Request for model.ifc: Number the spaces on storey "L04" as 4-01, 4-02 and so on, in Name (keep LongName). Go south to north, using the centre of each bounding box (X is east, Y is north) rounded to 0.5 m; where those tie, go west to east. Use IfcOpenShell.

First a look at what the model holds.

```python
import ifcopenshell
import ifcopenshell.util.element
import ifcopenshell.util.placement

model = ifcopenshell.open("model.ifc")
print(model.schema)
storey = next(s for s in model.by_type("IfcBuildingStorey") if s.Name == "L04")
spaces = [e for e in ifcopenshell.util.element.get_decomposition(storey) if e.is_a("IfcSpace")]
for e in sorted(spaces, key=lambda e: e.id()):
    origin = ifcopenshell.util.placement.get_local_placement(e.ObjectPlacement)[:3, 3]
    print(e.id(), e.Name, e.LongName, origin.round(2) + 0.0, sep=" | ")
```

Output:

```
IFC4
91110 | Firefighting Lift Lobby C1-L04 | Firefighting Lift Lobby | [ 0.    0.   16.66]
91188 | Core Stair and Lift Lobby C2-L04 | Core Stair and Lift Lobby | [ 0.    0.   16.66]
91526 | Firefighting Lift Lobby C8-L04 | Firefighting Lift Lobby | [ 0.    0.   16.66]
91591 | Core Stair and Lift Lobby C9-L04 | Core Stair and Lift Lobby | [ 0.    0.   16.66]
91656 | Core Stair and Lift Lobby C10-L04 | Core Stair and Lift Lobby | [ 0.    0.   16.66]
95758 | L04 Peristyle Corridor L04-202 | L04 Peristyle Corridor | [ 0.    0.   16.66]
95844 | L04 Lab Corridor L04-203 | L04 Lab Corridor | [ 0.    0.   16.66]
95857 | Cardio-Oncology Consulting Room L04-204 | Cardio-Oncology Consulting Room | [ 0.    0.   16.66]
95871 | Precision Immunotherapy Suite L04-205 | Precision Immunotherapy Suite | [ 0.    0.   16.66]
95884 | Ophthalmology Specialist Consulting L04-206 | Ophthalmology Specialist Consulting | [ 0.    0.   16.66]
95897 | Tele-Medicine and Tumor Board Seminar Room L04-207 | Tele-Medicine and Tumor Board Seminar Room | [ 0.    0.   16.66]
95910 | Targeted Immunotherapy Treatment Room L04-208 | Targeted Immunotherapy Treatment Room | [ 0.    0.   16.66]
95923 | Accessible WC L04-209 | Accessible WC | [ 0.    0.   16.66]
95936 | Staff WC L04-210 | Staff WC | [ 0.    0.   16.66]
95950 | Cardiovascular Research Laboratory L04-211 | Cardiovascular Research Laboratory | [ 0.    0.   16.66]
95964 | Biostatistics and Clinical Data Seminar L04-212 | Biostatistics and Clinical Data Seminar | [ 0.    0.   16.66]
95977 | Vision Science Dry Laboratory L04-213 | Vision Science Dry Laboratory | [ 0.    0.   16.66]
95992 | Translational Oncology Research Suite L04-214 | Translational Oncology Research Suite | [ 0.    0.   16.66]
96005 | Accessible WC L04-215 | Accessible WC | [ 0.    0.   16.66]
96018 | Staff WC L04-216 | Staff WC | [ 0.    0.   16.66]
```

```python
import ifcopenshell
import ifcopenshell.geom
import ifcopenshell.util.element
import ifcopenshell.util.shape

model = ifcopenshell.open("model.ifc")
settings = ifcopenshell.geom.settings()
settings.set("use-world-coords", True)


def centre(element):
    shape = ifcopenshell.geom.create_shape(settings, element)
    return ifcopenshell.util.shape.get_bbox_centroid(shape.geometry)


storey = next(s for s in model.by_type("IfcBuildingStorey") if s.Name == "L04")
spaces = [e for e in ifcopenshell.util.element.get_decomposition(storey) if e.is_a("IfcSpace")]

# Insertion points can sit at a corner or the storey origin, so sort by the geometry (in metres).
centres = {e: centre(e) for e in spaces}
spaces.sort(key=lambda e: (round(centres[e][1] / 0.5), centres[e][0]))

for i, e in enumerate(spaces, start=1):
    number = f"4-{i:02d}"
    e.Name = number
    print(e.id(), number)

model.write("model_v2.ifc")
```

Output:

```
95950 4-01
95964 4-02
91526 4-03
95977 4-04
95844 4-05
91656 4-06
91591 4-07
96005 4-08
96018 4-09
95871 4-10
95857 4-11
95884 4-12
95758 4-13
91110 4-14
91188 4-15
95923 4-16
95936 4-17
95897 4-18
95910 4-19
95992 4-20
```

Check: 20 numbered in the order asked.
